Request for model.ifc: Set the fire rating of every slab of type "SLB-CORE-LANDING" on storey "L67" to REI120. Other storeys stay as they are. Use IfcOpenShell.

First a look at what the model holds.

```python
import ifcopenshell
import ifcopenshell.util.element

model = ifcopenshell.open("model.ifc")
print(model.schema)
storey = next(s for s in model.by_type("IfcBuildingStorey") if s.Name == "L67")
slabs = [e for e in ifcopenshell.util.element.get_decomposition(storey) if e.is_a("IfcSlab")]
seen = {}
for e in slabs:
    element_type = ifcopenshell.util.element.get_type(e)
    key = (element_type.Name if element_type != e and element_type else None, ifcopenshell.util.element.get_pset(e, "Pset_SlabCommon", "FireRating"))
    seen[key] = seen.get(key, 0) + 1
for (name, value), count in sorted(seen.items(), key=str):
    print(count, "x", name, "|", value)
```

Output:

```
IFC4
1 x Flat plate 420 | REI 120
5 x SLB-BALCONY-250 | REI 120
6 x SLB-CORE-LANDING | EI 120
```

```python
import ifcopenshell
import ifcopenshell.api.pset
import ifcopenshell.util.element

model = ifcopenshell.open("model.ifc")

storey = next(s for s in model.by_type("IfcBuildingStorey") if s.Name == "L67")
slabs = [e for e in ifcopenshell.util.element.get_decomposition(storey) if e.is_a("IfcSlab")]

count = 0
for e in slabs:
    element_type = ifcopenshell.util.element.get_type(e)
    if element_type in (None, e) or element_type.Name != "SLB-CORE-LANDING":
        continue
    found = ifcopenshell.util.element.get_pset(e, "Pset_SlabCommon", should_inherit=False)
    if found:
        pset = model.by_id(found["id"])
        if len(ifcopenshell.util.element.get_elements_by_pset(pset)) > 1:
            pset = ifcopenshell.api.pset.unshare_pset(model, products=[e], pset=pset)[0]
    else:
        pset = ifcopenshell.api.pset.add_pset(model, product=e, name="Pset_SlabCommon")
    ifcopenshell.api.pset.edit_pset(model, pset=pset, properties={"FireRating": "REI120"})
    count += 1

print(count, "slabs updated")

model.write("model-out.ifc")
```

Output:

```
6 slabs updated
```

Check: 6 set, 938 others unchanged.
